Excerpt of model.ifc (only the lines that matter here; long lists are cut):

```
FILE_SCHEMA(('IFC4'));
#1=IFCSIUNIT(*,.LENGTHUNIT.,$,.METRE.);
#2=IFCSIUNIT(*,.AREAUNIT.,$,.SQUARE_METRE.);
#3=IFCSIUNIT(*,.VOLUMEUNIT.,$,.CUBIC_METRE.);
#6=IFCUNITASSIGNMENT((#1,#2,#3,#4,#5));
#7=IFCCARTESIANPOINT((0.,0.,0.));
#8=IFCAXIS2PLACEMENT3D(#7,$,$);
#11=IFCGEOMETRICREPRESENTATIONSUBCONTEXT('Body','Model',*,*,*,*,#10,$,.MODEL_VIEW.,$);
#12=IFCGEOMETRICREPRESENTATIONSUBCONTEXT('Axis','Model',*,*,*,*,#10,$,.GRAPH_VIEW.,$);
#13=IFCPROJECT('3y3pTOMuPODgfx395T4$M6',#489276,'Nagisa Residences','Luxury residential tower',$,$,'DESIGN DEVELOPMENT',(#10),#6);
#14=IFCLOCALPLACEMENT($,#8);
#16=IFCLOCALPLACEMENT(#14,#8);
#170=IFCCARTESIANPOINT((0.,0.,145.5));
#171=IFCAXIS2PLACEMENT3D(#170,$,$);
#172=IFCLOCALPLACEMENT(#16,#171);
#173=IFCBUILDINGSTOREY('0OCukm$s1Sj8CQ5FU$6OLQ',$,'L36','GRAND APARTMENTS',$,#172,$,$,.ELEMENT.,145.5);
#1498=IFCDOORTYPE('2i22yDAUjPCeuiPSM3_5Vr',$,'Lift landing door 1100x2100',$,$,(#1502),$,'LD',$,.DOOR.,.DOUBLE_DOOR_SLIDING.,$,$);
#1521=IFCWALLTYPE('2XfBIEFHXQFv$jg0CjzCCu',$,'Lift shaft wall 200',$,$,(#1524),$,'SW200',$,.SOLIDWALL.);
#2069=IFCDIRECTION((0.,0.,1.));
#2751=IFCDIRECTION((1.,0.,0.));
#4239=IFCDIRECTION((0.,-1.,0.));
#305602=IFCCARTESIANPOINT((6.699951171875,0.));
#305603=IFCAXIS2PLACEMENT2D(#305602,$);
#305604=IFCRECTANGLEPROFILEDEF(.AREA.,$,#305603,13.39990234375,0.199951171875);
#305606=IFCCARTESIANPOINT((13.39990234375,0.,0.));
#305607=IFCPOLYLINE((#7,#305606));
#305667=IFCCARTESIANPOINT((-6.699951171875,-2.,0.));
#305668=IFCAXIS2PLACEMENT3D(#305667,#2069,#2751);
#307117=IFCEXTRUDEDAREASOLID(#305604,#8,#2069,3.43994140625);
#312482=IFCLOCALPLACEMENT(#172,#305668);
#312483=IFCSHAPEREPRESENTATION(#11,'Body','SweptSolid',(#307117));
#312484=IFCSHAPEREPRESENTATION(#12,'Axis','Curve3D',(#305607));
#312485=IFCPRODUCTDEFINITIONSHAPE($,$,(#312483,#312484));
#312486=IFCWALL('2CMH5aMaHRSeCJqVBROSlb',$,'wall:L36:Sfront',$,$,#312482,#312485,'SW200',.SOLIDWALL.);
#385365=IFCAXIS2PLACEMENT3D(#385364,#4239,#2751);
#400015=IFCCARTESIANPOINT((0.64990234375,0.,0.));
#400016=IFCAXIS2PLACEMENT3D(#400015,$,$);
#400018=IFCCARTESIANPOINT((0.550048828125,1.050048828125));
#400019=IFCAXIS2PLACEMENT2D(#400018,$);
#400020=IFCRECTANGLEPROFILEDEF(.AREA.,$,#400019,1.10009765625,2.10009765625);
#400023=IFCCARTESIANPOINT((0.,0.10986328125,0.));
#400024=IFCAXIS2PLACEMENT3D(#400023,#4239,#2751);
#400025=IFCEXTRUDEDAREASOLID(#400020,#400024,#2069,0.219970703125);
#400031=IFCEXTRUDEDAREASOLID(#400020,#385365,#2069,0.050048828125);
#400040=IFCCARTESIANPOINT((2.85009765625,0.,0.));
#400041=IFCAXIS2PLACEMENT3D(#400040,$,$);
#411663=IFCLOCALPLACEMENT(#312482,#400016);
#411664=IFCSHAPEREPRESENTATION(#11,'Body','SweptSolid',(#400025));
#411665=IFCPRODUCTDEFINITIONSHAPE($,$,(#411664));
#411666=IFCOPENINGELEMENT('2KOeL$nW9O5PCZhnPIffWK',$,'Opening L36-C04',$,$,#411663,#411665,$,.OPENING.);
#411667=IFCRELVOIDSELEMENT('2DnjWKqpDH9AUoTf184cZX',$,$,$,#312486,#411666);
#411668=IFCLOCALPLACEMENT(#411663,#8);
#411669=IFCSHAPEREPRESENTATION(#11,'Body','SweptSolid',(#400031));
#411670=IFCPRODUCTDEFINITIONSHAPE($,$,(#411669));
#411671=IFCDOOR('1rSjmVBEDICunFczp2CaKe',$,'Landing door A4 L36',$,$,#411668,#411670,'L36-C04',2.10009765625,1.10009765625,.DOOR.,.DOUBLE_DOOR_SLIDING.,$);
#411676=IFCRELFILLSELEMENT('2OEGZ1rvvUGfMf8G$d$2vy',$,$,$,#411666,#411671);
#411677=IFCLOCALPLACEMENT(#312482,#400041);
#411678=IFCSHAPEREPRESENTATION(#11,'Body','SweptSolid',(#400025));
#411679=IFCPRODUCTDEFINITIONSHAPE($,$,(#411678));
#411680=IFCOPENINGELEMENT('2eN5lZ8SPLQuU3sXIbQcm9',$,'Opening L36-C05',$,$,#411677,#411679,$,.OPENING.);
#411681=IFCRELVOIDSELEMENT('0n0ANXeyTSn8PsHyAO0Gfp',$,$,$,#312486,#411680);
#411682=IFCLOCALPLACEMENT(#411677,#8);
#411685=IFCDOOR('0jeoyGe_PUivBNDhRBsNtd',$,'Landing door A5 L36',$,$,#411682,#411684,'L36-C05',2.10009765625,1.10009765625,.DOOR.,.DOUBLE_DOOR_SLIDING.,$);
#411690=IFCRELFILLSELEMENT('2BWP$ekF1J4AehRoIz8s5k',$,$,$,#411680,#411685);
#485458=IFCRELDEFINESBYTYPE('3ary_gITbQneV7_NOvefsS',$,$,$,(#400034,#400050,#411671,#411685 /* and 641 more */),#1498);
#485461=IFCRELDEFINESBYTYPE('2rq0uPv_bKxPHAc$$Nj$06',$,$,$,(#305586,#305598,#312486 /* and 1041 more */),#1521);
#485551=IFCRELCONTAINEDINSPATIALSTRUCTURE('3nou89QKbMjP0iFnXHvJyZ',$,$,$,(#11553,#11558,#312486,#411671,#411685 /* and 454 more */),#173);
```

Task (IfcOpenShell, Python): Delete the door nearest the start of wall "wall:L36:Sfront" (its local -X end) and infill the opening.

```python
import ifcopenshell
import ifcopenshell.api.feature
import ifcopenshell.api.root
import ifcopenshell.geom
import ifcopenshell.util.shape

model = ifcopenshell.open("model.ifc")
settings = ifcopenshell.geom.settings()


def volume(element):
    """Net volume in cubic metres, openings subtracted."""
    shape = ifcopenshell.geom.create_shape(settings, element)
    return ifcopenshell.util.shape.get_volume(shape.geometry)


door = model.by_guid("1rSjmVBEDICunFczp2CaKe")
opening = door.FillsVoids[0].RelatingOpeningElement
wall = opening.VoidsElements[0].RelatingBuildingElement
before = volume(wall)

ifcopenshell.api.root.remove_product(model, product=door)
ifcopenshell.api.feature.remove_feature(model, feature=opening)

after = volume(wall)

print(f"wall volume {before:.3f} -> {after:.3f} m3")

model.write("model-out.ifc")
```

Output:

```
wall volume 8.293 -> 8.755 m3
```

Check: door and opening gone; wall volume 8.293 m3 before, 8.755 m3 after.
